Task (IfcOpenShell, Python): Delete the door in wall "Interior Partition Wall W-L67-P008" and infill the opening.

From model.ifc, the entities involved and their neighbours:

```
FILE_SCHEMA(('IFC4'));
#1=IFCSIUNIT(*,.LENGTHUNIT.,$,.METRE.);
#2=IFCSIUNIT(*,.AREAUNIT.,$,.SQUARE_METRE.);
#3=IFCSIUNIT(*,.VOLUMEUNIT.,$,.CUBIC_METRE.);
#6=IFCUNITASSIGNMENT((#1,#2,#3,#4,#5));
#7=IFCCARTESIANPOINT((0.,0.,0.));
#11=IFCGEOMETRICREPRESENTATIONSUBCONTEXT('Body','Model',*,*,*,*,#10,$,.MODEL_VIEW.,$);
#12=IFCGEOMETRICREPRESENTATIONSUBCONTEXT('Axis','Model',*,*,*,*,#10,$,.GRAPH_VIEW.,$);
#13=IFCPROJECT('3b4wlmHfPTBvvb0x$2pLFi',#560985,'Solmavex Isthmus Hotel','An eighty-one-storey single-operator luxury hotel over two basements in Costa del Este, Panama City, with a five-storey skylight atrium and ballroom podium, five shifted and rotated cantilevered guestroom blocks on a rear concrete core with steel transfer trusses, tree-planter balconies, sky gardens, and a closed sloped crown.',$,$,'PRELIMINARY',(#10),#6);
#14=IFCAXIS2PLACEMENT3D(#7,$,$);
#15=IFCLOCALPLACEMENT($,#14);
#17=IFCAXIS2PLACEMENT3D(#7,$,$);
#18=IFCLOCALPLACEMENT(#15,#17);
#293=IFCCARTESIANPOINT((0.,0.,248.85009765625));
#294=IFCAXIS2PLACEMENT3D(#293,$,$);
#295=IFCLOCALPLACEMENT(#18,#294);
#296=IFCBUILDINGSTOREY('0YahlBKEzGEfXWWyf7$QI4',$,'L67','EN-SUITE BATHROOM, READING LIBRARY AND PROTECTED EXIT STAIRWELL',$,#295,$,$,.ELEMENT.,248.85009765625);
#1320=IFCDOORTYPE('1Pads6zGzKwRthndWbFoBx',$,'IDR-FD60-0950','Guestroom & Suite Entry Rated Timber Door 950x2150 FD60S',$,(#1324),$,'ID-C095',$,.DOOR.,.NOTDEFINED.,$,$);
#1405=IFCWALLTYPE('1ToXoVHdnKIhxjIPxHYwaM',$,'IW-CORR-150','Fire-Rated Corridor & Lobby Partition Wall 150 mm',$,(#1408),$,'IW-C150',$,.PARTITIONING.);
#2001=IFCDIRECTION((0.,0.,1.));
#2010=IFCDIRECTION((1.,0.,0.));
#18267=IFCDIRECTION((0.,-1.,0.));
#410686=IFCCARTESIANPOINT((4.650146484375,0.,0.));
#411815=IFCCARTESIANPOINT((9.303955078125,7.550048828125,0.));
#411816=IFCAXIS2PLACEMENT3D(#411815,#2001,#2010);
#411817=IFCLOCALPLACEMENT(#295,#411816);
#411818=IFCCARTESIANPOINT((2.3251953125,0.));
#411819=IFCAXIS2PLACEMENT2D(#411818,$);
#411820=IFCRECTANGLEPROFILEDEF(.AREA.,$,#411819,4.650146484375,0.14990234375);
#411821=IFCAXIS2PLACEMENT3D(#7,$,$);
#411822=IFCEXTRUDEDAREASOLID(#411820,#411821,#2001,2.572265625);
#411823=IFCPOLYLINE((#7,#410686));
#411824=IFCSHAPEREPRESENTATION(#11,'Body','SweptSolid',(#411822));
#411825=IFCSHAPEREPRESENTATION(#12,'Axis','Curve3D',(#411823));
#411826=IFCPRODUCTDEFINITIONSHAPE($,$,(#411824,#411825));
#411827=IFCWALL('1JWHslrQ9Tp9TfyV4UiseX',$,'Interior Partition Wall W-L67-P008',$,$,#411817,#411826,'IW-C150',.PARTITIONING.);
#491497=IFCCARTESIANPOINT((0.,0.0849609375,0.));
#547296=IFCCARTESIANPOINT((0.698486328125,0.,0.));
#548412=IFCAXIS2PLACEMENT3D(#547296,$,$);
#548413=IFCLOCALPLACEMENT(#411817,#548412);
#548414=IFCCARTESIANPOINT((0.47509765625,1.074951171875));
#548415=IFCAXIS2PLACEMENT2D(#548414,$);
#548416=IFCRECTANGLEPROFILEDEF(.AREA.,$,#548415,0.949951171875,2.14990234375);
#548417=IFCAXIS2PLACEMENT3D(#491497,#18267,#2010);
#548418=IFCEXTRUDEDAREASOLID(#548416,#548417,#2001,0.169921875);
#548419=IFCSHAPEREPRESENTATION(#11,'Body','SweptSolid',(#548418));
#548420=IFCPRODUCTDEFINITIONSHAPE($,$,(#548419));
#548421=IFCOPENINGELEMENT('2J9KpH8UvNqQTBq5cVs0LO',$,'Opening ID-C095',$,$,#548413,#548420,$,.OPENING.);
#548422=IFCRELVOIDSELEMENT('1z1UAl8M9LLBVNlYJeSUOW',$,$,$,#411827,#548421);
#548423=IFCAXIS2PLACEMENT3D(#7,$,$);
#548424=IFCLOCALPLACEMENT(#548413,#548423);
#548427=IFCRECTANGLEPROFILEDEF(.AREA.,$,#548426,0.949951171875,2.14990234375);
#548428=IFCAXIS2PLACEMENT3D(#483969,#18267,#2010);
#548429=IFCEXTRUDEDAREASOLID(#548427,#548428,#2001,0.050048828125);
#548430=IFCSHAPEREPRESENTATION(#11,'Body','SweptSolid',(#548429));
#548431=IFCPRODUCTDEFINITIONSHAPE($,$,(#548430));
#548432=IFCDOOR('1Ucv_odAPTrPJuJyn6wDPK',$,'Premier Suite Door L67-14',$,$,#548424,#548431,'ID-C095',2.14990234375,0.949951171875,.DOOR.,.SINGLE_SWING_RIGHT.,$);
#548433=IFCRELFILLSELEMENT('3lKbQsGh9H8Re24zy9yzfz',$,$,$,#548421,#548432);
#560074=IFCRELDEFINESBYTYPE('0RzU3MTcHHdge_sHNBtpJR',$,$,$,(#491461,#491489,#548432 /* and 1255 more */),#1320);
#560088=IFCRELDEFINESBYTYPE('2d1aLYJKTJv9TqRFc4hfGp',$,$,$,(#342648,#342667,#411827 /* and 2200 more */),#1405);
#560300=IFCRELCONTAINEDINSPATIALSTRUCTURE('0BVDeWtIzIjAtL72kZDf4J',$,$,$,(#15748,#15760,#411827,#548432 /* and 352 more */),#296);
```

```python
import ifcopenshell
import ifcopenshell.api.feature
import ifcopenshell.api.root
import ifcopenshell.geom
import ifcopenshell.util.shape

model = ifcopenshell.open("model.ifc")
settings = ifcopenshell.geom.settings()


def volume(element):
    """Net volume in cubic metres, openings subtracted."""
    shape = ifcopenshell.geom.create_shape(settings, element)
    return ifcopenshell.util.shape.get_volume(shape.geometry)


door = model.by_guid("1Ucv_odAPTrPJuJyn6wDPK")
opening = door.FillsVoids[0].RelatingOpeningElement
wall = opening.VoidsElements[0].RelatingBuildingElement
before = volume(wall)

ifcopenshell.api.root.remove_product(model, product=door)
ifcopenshell.api.feature.remove_feature(model, feature=opening)

after = volume(wall)

print(f"wall volume {before:.3f} -> {after:.3f} m3")

model.write("model_rev.ifc")
```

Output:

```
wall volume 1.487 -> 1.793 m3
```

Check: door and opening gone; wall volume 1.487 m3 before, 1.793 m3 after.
